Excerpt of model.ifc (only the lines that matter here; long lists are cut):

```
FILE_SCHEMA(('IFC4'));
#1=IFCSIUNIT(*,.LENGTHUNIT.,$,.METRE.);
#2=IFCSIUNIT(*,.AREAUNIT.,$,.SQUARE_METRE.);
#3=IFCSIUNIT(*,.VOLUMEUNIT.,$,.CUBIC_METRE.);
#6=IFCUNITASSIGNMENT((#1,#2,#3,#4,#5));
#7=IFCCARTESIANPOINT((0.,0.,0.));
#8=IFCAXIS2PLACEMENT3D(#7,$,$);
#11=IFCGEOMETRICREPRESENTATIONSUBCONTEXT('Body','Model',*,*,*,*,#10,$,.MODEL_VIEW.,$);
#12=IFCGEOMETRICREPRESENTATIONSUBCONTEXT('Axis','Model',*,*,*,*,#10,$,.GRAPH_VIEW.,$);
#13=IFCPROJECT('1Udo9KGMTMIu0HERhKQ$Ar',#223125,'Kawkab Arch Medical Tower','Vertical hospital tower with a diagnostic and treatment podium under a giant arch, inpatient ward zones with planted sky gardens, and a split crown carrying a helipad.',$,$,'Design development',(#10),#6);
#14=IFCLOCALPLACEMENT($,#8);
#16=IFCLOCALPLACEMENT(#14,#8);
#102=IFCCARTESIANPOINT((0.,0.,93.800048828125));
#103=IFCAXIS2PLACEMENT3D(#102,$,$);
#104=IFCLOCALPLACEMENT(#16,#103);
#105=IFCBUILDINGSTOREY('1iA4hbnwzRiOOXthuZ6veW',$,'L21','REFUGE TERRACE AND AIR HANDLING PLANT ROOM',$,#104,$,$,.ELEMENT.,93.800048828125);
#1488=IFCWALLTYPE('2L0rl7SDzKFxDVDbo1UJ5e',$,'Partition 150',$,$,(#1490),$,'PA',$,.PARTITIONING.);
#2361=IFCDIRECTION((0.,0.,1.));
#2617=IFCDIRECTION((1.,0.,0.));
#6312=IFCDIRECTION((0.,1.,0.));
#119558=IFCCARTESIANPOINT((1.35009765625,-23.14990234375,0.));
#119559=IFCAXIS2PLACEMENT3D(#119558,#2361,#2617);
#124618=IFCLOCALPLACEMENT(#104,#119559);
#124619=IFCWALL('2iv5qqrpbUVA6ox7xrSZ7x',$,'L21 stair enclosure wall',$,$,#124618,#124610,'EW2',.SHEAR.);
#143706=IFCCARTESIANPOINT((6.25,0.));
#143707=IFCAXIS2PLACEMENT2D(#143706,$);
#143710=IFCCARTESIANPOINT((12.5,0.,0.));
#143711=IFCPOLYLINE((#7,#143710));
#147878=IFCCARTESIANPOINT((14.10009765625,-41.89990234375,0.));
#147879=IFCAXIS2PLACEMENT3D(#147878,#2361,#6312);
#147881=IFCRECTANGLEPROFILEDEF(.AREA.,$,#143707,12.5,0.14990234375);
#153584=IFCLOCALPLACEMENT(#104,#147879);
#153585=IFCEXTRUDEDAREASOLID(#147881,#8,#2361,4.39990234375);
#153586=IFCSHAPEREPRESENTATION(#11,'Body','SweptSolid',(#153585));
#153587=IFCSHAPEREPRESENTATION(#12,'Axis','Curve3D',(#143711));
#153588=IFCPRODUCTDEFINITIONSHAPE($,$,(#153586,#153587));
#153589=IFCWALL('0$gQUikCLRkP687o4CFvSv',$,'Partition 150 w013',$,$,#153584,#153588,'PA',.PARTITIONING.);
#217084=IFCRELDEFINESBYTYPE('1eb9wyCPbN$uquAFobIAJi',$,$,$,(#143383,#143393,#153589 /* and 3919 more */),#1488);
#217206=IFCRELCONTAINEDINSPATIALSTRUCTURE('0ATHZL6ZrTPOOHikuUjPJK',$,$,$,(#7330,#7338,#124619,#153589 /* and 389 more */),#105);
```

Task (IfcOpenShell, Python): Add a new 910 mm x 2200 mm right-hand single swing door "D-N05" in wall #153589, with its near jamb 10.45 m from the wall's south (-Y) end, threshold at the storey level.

```python
import numpy as np
import ifcopenshell
import ifcopenshell.api.feature
import ifcopenshell.api.geometry
import ifcopenshell.api.root
import ifcopenshell.api.spatial
import ifcopenshell.geom
import ifcopenshell.util.element
import ifcopenshell.util.placement
import ifcopenshell.util.representation
import ifcopenshell.util.shape
import ifcopenshell.util.unit

model = ifcopenshell.open("model.ifc")
unit_scale = ifcopenshell.util.unit.calculate_unit_scale(model)
settings = ifcopenshell.geom.settings()


def volume(element):
    """Net volume in cubic metres, openings subtracted."""
    shape = ifcopenshell.geom.create_shape(settings, element)
    return ifcopenshell.util.shape.get_volume(shape.geometry)


wall = model.by_guid("0$gQUikCLRkP687o4CFvSv")
storey = ifcopenshell.util.element.get_container(wall, ifc_class="IfcBuildingStorey")
context = ifcopenshell.util.representation.get_context(model, "Model", "Body", "MODEL_VIEW")
before = volume(wall)

width, height, from_end, sill = 0.91, 2.2, 10.45, 0.0  # metres

# The wall runs along its own X axis, and the end named is its -X end.
wall_shape = ifcopenshell.geom.create_shape(settings, wall)
x, y, z = ifcopenshell.util.shape.get_vertices(wall_shape.geometry).T
start = x.min() + from_end
face, thickness = float(y.min()), float(y.max() - y.min())
wall_matrix = ifcopenshell.util.placement.get_local_placement(wall.ObjectPlacement)
level = ifcopenshell.util.placement.get_local_placement(storey.ObjectPlacement)[2, 3]


def in_wall(x, y):
    """Placement at x, y metres in the wall's axes, at sill height."""
    matrix = wall_matrix.copy()
    matrix[:, 3] = wall_matrix @ np.array([x / unit_scale, y / unit_scale, 0.0, 1.0])
    matrix[2, 3] = level + sill / unit_scale
    return matrix


# Opening: a box that overshoots both wall faces by 50 mm.
opening = ifcopenshell.api.root.create_entity(model, ifc_class="IfcOpeningElement", predefined_type="OPENING")
box = ifcopenshell.api.geometry.add_wall_representation(
    model, context=context, length=width, height=height, thickness=thickness + 0.1
)
ifcopenshell.api.geometry.assign_representation(model, product=opening, representation=box)
ifcopenshell.api.geometry.edit_object_placement(model, product=opening, matrix=in_wall(start, face - 0.05), is_si=False)
ifcopenshell.api.feature.add_feature(model, feature=opening, element=wall)

door = ifcopenshell.api.root.create_entity(model, ifc_class="IfcDoor", name="D-N05", predefined_type="DOOR")
door.OverallWidth, door.OverallHeight = width / unit_scale, height / unit_scale
door.OperationType = "SINGLE_SWING_RIGHT"
body = ifcopenshell.api.geometry.add_door_representation(
    model,
    context=context,
    overall_width=door.OverallWidth,
    overall_height=door.OverallHeight,
    operation_type="SINGLE_SWING_RIGHT",
    lining_properties={"LiningDepth": thickness / unit_scale, "ThresholdDepth": thickness / unit_scale},
)
ifcopenshell.api.geometry.assign_representation(model, product=door, representation=body)
ifcopenshell.api.spatial.assign_container(model, products=[door], relating_structure=storey)
ifcopenshell.api.feature.add_filling(model, opening=opening, element=door)

# The lining spans the wall, so the door starts at the wall face.
ifcopenshell.api.geometry.edit_object_placement(model, product=door, matrix=in_wall(start, face), is_si=False)

after = volume(wall)

print(f"wall volume {before:.3f} -> {after:.3f} m3")

model.write("model_edited.ifc")
```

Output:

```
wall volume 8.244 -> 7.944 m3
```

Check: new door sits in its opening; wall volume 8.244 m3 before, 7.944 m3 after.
